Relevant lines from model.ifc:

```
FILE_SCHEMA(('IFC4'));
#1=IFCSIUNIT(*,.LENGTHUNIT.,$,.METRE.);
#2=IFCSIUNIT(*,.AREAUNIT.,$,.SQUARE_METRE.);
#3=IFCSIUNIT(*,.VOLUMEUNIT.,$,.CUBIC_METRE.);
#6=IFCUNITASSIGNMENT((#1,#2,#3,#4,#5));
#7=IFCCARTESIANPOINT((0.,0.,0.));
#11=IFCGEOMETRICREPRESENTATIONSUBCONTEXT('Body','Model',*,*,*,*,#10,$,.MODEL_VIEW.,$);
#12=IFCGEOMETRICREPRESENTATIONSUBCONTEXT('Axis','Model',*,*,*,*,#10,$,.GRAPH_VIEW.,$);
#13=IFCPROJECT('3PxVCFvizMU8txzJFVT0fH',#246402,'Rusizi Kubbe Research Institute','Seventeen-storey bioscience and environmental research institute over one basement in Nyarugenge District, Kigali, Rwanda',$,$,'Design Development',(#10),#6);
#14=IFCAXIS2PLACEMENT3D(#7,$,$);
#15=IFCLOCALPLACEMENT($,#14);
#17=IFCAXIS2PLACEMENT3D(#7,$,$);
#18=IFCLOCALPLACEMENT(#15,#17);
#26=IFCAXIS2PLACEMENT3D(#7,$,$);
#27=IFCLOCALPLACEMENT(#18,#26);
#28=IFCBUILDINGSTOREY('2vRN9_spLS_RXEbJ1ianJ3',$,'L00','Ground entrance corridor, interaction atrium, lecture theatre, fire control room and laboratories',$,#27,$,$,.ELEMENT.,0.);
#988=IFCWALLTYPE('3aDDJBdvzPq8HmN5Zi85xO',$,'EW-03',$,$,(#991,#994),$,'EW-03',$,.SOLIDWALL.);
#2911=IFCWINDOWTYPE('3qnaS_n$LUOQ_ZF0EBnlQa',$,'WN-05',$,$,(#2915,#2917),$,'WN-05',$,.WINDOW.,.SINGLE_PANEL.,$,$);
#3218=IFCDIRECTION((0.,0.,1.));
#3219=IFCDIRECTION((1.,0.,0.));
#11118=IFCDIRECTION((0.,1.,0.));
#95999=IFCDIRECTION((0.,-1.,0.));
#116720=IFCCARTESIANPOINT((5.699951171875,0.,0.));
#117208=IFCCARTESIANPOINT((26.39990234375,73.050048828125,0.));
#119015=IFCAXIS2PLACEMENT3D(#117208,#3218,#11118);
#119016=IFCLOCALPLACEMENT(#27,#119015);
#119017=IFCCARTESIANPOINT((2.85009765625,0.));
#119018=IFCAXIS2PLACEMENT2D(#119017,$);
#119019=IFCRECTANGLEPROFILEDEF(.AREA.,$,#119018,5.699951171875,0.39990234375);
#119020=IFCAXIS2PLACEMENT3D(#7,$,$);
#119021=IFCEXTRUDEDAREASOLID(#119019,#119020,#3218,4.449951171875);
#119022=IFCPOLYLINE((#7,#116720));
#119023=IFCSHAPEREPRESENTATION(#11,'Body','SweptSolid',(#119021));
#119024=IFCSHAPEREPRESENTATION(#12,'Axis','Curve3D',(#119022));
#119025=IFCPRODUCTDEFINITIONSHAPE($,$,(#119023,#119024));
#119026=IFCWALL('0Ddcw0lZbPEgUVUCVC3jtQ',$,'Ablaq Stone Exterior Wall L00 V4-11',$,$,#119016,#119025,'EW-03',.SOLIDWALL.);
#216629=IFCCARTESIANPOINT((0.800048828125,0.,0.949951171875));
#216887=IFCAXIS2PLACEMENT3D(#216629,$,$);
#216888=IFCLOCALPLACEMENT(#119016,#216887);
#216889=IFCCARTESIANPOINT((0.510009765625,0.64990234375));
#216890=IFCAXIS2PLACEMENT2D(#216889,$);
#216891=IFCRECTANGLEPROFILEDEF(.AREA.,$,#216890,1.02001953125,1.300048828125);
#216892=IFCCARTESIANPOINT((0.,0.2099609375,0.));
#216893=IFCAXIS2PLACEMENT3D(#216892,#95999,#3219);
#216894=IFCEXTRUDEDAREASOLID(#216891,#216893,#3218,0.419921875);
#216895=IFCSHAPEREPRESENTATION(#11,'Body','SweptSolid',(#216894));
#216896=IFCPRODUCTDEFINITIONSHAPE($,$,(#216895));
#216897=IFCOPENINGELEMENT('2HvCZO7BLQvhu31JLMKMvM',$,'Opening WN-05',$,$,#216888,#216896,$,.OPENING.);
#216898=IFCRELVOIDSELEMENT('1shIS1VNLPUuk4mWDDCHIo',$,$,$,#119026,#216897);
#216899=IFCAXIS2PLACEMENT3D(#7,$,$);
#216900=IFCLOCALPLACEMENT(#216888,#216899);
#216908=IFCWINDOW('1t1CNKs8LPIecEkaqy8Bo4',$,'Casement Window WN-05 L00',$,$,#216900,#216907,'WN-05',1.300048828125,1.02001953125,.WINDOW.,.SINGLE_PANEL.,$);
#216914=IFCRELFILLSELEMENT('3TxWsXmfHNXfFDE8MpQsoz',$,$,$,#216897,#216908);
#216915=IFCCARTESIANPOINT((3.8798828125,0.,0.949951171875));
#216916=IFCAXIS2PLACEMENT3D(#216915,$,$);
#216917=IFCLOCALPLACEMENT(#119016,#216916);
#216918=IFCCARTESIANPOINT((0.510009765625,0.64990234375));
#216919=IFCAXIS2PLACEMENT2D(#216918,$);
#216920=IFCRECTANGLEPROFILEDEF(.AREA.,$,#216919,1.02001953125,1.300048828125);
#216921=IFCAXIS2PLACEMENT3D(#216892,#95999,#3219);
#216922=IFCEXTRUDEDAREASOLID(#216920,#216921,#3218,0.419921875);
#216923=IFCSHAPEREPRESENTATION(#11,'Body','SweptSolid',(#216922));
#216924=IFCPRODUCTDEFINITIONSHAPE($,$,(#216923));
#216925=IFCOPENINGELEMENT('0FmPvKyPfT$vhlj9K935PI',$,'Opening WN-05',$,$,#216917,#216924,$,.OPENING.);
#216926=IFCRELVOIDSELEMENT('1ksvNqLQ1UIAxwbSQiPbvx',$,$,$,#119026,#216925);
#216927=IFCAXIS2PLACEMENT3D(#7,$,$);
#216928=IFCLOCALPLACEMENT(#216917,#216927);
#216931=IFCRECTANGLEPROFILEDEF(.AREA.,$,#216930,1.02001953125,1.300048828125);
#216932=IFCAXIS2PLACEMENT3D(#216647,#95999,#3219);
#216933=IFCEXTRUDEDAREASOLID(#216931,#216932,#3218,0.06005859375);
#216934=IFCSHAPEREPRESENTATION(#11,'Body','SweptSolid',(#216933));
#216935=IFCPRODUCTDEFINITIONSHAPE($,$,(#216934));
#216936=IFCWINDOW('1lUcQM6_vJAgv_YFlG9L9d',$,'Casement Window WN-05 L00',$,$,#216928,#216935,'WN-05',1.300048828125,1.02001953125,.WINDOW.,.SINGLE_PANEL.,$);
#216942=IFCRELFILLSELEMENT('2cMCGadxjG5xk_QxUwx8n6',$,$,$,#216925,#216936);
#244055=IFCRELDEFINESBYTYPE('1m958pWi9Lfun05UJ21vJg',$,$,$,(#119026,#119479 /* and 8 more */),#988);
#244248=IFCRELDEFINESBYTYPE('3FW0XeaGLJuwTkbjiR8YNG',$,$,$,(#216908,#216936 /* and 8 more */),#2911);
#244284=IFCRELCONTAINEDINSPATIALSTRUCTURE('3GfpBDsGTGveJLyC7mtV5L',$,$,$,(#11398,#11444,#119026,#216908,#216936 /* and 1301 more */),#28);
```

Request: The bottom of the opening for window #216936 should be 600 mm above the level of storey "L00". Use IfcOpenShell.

```python
import numpy as np
import ifcopenshell
import ifcopenshell.api.geometry
import ifcopenshell.geom
import ifcopenshell.util.element
import ifcopenshell.util.placement
import ifcopenshell.util.shape
import ifcopenshell.util.unit

model = ifcopenshell.open("model.ifc")
unit_scale = ifcopenshell.util.unit.calculate_unit_scale(model)

window = model.by_guid("1lUcQM6_vJAgv_YFlG9L9d")
opening = window.FillsVoids[0].RelatingOpeningElement
storey = ifcopenshell.util.element.get_container(window, ifc_class="IfcBuildingStorey")
level = ifcopenshell.util.placement.get_local_placement(storey.ObjectPlacement)[2, 3]

# The opening's origin need not be at the sill, so measure its lowest point.
shape = ifcopenshell.geom.create_shape(ifcopenshell.geom.settings(), opening)
bottom = ifcopenshell.util.shape.get_shape_bottom_elevation(shape, shape.geometry) / unit_scale
dz = level + 0.6 / unit_scale - bottom

shift = np.array([0.0, 0.0, dz])
# The window is placed relative to its opening, so it follows when the opening moves.
matrix = ifcopenshell.util.placement.get_local_placement(opening.ObjectPlacement)
matrix[:3, 3] += shift
ifcopenshell.api.geometry.edit_object_placement(
    model, product=opening, matrix=matrix, is_si=False, should_transform_children=True
)

print(f"moved by {dz * unit_scale:+.3f} m")

model.write("model_updated.ifc")
```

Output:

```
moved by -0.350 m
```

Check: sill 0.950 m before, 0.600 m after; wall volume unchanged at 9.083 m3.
